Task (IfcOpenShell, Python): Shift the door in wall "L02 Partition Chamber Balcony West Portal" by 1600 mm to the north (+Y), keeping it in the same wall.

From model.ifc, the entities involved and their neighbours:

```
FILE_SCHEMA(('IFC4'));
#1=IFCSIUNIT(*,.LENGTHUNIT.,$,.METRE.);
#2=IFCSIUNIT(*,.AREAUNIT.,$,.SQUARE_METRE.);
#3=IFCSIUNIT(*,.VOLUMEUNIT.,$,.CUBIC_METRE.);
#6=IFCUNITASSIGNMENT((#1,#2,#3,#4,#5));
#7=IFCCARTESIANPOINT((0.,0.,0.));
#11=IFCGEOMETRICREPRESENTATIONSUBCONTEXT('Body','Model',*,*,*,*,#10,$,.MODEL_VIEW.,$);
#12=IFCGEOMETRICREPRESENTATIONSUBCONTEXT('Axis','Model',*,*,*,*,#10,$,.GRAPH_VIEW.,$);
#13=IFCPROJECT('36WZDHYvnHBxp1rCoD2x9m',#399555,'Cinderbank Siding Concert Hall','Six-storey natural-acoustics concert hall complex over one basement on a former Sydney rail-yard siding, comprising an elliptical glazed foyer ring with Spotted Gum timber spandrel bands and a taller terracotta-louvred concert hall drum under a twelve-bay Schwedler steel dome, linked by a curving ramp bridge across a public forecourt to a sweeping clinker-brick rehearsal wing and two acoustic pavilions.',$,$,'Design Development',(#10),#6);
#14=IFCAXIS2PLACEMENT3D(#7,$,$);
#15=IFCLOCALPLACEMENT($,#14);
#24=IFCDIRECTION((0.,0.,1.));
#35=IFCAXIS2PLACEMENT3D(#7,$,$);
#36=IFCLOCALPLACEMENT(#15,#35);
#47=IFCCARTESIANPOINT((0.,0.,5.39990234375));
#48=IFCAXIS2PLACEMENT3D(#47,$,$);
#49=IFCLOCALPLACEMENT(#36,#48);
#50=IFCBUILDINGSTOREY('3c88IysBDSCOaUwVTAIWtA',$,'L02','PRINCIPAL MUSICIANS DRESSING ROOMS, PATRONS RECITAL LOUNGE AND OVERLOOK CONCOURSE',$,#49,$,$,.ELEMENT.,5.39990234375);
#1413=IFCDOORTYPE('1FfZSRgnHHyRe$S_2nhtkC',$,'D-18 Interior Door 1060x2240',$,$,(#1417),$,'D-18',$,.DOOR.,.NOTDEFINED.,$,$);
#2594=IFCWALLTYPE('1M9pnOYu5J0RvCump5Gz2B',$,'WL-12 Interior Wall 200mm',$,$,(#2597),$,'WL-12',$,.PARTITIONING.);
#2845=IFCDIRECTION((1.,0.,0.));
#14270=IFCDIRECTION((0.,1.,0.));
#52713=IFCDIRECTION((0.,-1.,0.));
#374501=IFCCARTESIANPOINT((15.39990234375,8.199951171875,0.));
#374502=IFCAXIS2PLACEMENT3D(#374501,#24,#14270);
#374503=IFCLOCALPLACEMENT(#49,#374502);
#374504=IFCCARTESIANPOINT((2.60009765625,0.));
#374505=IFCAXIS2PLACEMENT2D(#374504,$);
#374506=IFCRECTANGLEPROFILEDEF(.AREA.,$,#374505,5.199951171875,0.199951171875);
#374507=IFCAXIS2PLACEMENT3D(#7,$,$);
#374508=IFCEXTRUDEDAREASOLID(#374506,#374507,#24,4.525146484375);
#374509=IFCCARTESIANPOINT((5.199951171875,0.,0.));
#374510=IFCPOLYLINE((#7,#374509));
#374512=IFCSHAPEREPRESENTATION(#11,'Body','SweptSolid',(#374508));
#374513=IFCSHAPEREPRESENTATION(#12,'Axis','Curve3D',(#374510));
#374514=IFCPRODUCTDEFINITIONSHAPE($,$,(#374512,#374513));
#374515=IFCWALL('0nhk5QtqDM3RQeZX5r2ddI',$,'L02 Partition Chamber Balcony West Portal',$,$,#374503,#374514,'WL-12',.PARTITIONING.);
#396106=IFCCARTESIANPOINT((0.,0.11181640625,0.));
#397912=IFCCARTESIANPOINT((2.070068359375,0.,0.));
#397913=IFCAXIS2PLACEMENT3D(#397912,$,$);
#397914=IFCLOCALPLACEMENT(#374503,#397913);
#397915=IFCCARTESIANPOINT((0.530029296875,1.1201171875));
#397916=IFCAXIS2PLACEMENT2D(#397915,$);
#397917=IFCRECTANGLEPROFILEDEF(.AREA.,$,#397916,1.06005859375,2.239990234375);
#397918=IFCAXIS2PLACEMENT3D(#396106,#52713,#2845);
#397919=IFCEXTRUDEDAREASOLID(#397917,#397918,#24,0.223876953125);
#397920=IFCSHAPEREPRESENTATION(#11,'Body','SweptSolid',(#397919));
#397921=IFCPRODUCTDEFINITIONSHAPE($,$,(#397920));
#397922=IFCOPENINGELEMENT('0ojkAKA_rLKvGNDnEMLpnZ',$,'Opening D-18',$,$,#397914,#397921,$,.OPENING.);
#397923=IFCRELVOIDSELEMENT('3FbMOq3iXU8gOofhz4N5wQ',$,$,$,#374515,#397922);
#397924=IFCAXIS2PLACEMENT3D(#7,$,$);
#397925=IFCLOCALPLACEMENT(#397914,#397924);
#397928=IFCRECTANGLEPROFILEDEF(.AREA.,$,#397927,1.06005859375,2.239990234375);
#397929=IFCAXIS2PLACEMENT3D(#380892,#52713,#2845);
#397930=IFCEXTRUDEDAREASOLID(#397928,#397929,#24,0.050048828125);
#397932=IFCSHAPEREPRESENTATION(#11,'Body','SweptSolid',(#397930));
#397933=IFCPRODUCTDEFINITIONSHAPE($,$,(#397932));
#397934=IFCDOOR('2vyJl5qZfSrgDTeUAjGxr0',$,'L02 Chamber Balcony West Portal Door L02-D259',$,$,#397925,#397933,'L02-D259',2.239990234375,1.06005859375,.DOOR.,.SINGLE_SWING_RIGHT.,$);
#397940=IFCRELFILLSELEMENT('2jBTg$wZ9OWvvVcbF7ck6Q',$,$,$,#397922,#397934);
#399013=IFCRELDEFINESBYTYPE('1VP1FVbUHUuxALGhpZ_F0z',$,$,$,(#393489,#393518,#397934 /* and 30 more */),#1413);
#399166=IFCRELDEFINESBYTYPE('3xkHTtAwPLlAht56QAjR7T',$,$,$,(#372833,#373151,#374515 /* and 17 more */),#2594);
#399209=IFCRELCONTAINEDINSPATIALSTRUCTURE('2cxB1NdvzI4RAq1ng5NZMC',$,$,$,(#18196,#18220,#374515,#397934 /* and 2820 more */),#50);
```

```python
import ifcopenshell
import ifcopenshell.api.geometry
import ifcopenshell.util.placement
import ifcopenshell.util.unit

model = ifcopenshell.open("model.ifc")
unit_scale = ifcopenshell.util.unit.calculate_unit_scale(model)

door = model.by_id(397934)
opening = door.FillsVoids[0].RelatingOpeningElement
wall = opening.VoidsElements[0].RelatingBuildingElement

wall_matrix = ifcopenshell.util.placement.get_local_placement(wall.ObjectPlacement)
shift = wall_matrix[:3, 0] * 1.6 / unit_scale
before = ifcopenshell.util.placement.get_local_placement(door.ObjectPlacement)[:3, 3].copy()

# The door is placed relative to its opening, so it follows when the opening moves.
matrix = ifcopenshell.util.placement.get_local_placement(opening.ObjectPlacement)
matrix[:3, 3] += shift
ifcopenshell.api.geometry.edit_object_placement(
    model, product=opening, matrix=matrix, is_si=False, should_transform_children=True
)

after = ifcopenshell.util.placement.get_local_placement(door.ObjectPlacement)[:3, 3]
print("door moved by", (after - before).round(3) + 0.0)

model.write("model_edited.ifc")
```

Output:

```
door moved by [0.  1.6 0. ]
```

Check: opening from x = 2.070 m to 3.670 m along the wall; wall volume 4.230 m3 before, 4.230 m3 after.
